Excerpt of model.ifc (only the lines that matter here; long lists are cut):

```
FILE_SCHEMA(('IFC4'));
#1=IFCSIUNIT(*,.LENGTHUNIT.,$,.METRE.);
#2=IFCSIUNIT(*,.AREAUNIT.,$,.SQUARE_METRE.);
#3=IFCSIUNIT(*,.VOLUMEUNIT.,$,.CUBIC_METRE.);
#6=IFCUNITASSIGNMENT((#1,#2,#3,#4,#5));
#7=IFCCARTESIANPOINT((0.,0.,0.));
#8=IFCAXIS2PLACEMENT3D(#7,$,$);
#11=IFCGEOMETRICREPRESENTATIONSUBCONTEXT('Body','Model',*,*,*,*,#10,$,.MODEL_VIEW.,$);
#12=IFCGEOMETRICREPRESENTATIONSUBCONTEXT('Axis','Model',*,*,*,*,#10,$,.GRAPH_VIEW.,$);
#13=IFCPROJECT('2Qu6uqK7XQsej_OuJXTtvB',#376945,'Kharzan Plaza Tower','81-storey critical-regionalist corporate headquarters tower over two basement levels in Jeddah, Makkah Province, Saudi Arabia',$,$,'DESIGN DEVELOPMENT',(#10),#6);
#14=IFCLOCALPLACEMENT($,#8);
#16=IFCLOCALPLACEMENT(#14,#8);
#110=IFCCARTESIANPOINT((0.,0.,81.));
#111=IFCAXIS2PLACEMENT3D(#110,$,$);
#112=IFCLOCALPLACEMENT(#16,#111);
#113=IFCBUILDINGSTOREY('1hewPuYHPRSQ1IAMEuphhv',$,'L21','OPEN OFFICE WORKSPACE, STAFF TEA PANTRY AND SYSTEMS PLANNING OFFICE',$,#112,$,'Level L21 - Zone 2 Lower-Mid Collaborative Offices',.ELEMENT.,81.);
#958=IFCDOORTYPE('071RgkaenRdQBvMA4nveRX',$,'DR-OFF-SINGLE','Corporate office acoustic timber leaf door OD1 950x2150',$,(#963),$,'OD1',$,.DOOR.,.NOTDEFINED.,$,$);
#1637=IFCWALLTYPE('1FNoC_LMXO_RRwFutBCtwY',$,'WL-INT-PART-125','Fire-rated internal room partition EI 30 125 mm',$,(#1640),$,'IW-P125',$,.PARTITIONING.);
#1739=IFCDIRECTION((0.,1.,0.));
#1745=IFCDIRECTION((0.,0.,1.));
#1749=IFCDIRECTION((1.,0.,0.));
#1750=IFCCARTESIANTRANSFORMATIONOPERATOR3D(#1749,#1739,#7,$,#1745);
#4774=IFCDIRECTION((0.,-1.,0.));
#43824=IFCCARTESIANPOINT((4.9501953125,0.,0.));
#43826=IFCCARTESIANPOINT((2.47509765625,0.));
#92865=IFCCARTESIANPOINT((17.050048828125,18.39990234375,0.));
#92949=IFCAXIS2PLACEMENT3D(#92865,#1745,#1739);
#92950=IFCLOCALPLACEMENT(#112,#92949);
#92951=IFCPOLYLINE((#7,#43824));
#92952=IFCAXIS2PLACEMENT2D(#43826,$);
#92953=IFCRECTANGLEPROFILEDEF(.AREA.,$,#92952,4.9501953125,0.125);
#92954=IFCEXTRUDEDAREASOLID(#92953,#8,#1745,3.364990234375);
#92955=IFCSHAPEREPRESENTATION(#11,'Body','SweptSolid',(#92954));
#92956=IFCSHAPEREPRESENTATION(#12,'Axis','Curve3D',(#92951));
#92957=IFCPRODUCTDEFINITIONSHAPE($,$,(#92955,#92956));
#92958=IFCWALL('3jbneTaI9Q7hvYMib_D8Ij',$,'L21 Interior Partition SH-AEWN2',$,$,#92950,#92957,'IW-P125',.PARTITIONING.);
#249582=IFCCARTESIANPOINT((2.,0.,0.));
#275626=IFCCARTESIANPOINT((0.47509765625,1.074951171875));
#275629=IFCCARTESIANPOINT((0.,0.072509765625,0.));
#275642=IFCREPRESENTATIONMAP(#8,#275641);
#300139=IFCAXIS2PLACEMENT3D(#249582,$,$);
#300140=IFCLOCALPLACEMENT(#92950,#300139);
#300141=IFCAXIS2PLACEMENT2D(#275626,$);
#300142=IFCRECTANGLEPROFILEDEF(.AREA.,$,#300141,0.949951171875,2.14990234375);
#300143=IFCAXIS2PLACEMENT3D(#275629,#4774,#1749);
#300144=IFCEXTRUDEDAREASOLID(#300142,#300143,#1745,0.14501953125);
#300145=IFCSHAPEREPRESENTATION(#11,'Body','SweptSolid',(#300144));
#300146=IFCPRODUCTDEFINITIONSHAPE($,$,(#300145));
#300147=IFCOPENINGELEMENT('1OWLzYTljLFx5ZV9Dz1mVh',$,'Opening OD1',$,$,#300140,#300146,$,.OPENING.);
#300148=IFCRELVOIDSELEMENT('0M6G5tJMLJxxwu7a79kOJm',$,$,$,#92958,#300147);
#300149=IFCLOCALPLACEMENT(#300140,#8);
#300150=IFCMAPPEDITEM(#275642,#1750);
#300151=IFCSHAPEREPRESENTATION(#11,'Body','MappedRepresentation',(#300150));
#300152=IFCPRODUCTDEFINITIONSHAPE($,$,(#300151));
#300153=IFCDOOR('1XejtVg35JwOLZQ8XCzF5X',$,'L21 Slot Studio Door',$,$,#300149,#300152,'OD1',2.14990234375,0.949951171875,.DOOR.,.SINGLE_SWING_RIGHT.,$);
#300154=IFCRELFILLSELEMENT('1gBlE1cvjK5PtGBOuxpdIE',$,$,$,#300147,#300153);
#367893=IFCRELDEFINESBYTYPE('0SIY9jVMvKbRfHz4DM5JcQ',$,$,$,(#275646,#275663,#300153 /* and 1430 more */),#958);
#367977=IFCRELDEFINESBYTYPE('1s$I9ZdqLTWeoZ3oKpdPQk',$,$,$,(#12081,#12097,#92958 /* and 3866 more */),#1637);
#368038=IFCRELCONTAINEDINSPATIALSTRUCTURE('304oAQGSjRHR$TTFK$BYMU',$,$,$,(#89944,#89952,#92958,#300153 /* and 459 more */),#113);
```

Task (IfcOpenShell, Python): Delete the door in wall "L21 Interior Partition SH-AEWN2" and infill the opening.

```python
import ifcopenshell
import ifcopenshell.api.feature
import ifcopenshell.api.root
import ifcopenshell.geom
import ifcopenshell.util.shape

model = ifcopenshell.open("model.ifc")
settings = ifcopenshell.geom.settings()


def volume(element):
    """Net volume in cubic metres, openings subtracted."""
    shape = ifcopenshell.geom.create_shape(settings, element)
    return ifcopenshell.util.shape.get_volume(shape.geometry)


door = model.by_guid("1XejtVg35JwOLZQ8XCzF5X")
opening = door.FillsVoids[0].RelatingOpeningElement
wall = opening.VoidsElements[0].RelatingBuildingElement
before = volume(wall)

ifcopenshell.api.root.remove_product(model, product=door)
ifcopenshell.api.feature.remove_feature(model, feature=opening)

after = volume(wall)

print(f"wall volume {before:.3f} -> {after:.3f} m3")

model.write("model_v2.ifc")
```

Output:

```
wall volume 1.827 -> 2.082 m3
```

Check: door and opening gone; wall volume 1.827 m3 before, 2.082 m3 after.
